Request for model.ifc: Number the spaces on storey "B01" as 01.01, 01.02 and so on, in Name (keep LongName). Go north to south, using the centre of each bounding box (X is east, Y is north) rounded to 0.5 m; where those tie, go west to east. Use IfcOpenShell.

First a look at what the model holds.

```python
import ifcopenshell
import ifcopenshell.util.element
import ifcopenshell.util.placement

model = ifcopenshell.open("model.ifc")
print(model.schema)
storey = next(s for s in model.by_type("IfcBuildingStorey") if s.Name == "B01")
spaces = [e for e in ifcopenshell.util.element.get_decomposition(storey) if e.is_a("IfcSpace")]
for e in sorted(spaces, key=lambda e: e.id()):
    origin = ifcopenshell.util.placement.get_local_placement(e.ObjectPlacement)[:3, 3]
    print(e.id(), e.Name, e.LongName, origin.round(2) + 0.0, sep=" | ")
```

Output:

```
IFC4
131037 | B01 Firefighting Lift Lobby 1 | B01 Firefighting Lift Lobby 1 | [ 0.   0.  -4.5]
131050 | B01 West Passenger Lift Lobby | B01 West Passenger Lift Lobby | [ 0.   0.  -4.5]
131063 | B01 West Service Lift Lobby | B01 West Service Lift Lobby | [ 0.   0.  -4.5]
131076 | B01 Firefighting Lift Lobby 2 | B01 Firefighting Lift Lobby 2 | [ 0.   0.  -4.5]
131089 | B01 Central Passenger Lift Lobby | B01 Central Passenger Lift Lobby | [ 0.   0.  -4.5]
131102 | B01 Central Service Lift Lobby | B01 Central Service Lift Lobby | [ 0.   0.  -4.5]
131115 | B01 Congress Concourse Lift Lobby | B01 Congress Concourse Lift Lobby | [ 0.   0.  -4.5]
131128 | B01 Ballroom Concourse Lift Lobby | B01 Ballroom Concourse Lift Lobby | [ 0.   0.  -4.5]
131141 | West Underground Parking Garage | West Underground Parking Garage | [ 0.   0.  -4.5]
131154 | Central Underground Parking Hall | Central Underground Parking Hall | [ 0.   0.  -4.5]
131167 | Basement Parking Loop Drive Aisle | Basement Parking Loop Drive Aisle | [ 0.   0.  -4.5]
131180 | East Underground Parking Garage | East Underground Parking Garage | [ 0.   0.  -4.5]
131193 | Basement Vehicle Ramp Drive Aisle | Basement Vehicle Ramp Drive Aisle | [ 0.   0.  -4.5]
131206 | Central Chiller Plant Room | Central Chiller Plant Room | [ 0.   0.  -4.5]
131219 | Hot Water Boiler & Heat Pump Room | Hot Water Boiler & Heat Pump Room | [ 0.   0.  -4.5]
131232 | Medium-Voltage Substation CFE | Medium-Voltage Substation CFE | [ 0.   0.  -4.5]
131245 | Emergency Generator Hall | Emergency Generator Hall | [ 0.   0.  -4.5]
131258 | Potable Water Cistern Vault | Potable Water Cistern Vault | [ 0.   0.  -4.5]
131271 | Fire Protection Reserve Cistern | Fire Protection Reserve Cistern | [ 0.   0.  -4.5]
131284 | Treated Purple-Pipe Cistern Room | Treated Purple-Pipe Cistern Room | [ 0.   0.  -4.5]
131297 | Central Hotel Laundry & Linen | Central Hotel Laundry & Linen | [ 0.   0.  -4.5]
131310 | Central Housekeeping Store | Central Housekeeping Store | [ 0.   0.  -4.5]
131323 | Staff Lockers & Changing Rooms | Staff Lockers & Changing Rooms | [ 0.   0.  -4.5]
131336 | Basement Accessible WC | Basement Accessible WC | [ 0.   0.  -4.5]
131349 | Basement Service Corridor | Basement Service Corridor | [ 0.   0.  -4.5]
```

```python
import ifcopenshell
import ifcopenshell.geom
import ifcopenshell.util.element
import ifcopenshell.util.shape

model = ifcopenshell.open("model.ifc")
settings = ifcopenshell.geom.settings()
settings.set("use-world-coords", True)


def centre(element):
    shape = ifcopenshell.geom.create_shape(settings, element)
    return ifcopenshell.util.shape.get_bbox_centroid(shape.geometry)


storey = next(s for s in model.by_type("IfcBuildingStorey") if s.Name == "B01")
spaces = [e for e in ifcopenshell.util.element.get_decomposition(storey) if e.is_a("IfcSpace")]

# Insertion points can sit at a corner or the storey origin, so sort by the geometry (in metres).
centres = {e: centre(e) for e in spaces}
spaces.sort(key=lambda e: (-round(centres[e][1] / 0.5), centres[e][0]))

for i, e in enumerate(spaces, start=1):
    number = f"01.{i:02d}"
    e.Name = number
    print(e.id(), number)

model.write("model-out.ifc")
```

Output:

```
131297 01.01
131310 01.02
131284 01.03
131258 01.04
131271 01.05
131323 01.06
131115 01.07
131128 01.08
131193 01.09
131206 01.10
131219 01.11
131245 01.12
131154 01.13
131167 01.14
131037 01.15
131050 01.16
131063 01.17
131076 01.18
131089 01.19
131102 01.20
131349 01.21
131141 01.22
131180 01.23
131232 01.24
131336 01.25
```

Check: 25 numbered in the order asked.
